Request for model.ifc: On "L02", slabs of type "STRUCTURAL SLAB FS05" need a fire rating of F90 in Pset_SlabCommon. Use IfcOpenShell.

First a look at what the model holds.

```python
import ifcopenshell
import ifcopenshell.util.element

model = ifcopenshell.open("model.ifc")
print(model.schema)
storey = next(s for s in model.by_type("IfcBuildingStorey") if s.Name == "L02")
slabs = [e for e in ifcopenshell.util.element.get_decomposition(storey) if e.is_a("IfcSlab")]
seen = {}
for e in slabs:
    element_type = ifcopenshell.util.element.get_type(e)
    key = (element_type.Name if element_type != e and element_type else None, ifcopenshell.util.element.get_pset(e, "Pset_SlabCommon", "FireRating"))
    seen[key] = seen.get(key, 0) + 1
for (name, value), count in sorted(seen.items(), key=str):
    print(count, "x", name, "|", value)
```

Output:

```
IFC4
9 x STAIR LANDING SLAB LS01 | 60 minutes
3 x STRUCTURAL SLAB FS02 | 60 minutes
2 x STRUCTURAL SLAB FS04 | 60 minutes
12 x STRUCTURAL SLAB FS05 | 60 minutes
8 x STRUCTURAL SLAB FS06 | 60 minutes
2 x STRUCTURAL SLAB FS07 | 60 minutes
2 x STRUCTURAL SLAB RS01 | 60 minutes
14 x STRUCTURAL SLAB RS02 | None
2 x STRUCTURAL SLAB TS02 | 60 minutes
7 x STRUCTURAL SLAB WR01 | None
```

```python
import ifcopenshell
import ifcopenshell.api.pset
import ifcopenshell.util.element

model = ifcopenshell.open("model.ifc")

storey = next(s for s in model.by_type("IfcBuildingStorey") if s.Name == "L02")
slabs = [e for e in ifcopenshell.util.element.get_decomposition(storey) if e.is_a("IfcSlab")]

count = 0
for e in slabs:
    element_type = ifcopenshell.util.element.get_type(e)
    if element_type in (None, e) or element_type.Name != "STRUCTURAL SLAB FS05":
        continue
    # add_pset returns the element's existing set when there is one.
    pset = ifcopenshell.api.pset.add_pset(model, product=e, name="Pset_SlabCommon")
    ifcopenshell.api.pset.edit_pset(model, pset=pset, properties={"FireRating": "F90"})
    count += 1

print(count, "slabs updated")

model.write("model_updated.ifc")
```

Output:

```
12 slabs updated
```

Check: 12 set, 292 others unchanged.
